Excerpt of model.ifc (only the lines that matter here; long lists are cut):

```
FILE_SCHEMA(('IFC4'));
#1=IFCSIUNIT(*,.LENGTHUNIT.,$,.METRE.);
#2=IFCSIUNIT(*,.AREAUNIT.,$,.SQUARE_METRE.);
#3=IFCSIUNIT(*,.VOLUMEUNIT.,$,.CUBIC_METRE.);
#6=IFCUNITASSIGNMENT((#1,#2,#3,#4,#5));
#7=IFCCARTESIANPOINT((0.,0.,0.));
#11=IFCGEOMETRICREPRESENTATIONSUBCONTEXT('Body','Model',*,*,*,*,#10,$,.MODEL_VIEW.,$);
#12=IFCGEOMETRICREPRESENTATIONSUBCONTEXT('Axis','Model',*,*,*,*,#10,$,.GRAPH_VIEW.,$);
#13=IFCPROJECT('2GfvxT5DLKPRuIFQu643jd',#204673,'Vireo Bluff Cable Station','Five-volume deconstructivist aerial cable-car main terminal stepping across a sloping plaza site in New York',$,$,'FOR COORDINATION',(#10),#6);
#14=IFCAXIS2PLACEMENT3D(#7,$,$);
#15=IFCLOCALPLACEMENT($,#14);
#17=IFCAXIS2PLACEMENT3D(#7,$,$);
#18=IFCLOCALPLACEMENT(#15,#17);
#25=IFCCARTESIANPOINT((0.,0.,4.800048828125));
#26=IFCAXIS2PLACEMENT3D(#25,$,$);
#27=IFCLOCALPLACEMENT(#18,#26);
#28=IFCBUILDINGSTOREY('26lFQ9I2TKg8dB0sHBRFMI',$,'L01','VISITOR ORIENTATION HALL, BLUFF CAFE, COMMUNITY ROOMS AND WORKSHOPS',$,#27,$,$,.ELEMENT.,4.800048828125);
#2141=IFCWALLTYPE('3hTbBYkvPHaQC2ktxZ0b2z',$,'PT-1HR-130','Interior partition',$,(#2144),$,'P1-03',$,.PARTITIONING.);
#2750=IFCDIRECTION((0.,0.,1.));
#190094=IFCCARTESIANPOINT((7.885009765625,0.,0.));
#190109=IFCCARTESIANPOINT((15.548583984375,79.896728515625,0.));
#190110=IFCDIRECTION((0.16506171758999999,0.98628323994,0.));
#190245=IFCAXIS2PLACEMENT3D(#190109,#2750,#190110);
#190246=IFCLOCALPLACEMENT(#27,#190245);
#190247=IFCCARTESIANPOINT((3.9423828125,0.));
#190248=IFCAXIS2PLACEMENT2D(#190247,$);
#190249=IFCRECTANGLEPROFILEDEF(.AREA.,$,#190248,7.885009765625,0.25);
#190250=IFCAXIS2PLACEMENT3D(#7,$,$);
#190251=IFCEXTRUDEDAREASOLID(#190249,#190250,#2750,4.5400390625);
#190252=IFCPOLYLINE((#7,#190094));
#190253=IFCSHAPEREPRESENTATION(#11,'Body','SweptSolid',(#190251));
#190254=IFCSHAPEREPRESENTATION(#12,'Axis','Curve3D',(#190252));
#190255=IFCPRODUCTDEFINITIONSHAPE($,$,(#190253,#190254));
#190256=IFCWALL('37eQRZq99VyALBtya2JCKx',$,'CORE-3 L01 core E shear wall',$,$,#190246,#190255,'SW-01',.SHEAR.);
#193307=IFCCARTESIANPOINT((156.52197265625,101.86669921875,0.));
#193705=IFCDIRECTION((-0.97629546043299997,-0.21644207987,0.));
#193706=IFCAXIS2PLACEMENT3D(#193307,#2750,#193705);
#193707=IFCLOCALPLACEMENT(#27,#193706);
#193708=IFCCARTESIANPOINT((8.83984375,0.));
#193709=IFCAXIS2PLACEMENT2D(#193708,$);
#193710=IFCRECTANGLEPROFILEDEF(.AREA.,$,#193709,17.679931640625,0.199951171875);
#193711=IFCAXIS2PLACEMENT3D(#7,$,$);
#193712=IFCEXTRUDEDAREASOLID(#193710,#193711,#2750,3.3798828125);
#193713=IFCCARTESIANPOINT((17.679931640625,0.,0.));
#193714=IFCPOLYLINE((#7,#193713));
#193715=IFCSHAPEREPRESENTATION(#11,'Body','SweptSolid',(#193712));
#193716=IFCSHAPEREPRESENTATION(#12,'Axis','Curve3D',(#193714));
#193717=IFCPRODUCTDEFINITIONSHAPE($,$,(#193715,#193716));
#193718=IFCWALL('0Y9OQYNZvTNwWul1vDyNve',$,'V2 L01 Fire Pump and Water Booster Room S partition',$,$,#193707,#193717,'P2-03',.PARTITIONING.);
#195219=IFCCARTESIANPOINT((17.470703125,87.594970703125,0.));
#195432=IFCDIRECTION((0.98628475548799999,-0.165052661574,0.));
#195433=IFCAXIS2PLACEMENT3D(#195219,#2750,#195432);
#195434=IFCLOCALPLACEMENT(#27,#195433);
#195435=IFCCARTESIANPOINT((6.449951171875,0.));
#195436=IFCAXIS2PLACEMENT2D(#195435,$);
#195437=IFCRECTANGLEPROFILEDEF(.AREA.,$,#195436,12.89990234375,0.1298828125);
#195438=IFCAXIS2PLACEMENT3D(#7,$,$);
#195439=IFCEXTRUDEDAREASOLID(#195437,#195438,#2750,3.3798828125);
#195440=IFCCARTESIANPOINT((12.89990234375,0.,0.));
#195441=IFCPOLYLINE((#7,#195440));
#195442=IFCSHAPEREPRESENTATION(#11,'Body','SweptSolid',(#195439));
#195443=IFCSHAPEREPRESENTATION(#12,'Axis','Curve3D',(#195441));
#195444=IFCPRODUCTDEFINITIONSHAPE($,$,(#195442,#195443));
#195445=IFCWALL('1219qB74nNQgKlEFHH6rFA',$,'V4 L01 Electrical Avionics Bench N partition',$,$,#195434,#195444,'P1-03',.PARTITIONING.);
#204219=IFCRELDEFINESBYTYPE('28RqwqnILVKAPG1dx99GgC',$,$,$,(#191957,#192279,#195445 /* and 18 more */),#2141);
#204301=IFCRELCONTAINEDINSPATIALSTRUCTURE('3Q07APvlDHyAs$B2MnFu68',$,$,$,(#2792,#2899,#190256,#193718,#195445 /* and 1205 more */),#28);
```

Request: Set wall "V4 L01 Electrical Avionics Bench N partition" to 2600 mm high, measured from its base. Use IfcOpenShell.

```python
import ifcopenshell
import ifcopenshell.geom
import ifcopenshell.util.representation
import ifcopenshell.util.shape

model = ifcopenshell.open("model.ifc")
settings = ifcopenshell.geom.settings()


def volume(element):
    """Net volume in cubic metres, openings subtracted."""
    shape = ifcopenshell.geom.create_shape(settings, element)
    return ifcopenshell.util.shape.get_volume(shape.geometry)


wall = model.by_id(195445)
before = volume(wall)

body = ifcopenshell.util.representation.get_representation(wall, "Model", "Body")
solid = body.Items[0]
old_height = solid.Depth
solid.Depth = 2.6
after = volume(wall)

print(f"height {old_height:g} -> {solid.Depth:g}, volume {before:.3f} -> {after:.3f} m3")

model.write("model_v2.ifc")
```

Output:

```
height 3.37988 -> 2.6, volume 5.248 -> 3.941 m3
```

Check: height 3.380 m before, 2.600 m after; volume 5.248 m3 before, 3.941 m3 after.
